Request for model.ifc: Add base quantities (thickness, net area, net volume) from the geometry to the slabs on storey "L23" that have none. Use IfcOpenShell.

First a look at what the model holds.

```python
import ifcopenshell
import ifcopenshell.util.element
import ifcopenshell.util.unit

model = ifcopenshell.open("model.ifc")
print(model.schema)
for unit_type in ("LENGTHUNIT", "AREAUNIT", "VOLUMEUNIT"):
    print(unit_type, ifcopenshell.util.unit.calculate_unit_scale(model, unit_type))
storey = next(s for s in model.by_type("IfcBuildingStorey") if s.Name == "L23")
slabs = [e for e in ifcopenshell.util.element.get_decomposition(storey) if e.is_a("IfcSlab")]
for e in sorted(slabs, key=lambda e: e.id()):
    print(e.id(), e.is_a(), e.Name, list(ifcopenshell.util.element.get_psets(e, qtos_only=True)), sep=" | ")
```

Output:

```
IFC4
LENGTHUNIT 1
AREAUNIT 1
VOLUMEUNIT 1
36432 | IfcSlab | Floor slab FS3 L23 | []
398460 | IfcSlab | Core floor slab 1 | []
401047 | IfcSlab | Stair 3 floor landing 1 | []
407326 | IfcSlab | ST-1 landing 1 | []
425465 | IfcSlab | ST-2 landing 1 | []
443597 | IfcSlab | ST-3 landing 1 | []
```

```python
import ifcopenshell
import ifcopenshell.api.pset
import ifcopenshell.geom
import ifcopenshell.util.element
import ifcopenshell.util.shape
import ifcopenshell.util.unit

model = ifcopenshell.open("model.ifc")
unit_scale = ifcopenshell.util.unit.calculate_unit_scale(model)
area_scale = ifcopenshell.util.unit.calculate_unit_scale(model, "AREAUNIT")
volume_scale = ifcopenshell.util.unit.calculate_unit_scale(model, "VOLUMEUNIT")
settings = ifcopenshell.geom.settings()

storey = next(s for s in model.by_type("IfcBuildingStorey") if s.Name == "L23")
slabs = [e for e in ifcopenshell.util.element.get_decomposition(storey) if e.is_a("IfcSlab")]

for e in sorted(slabs, key=lambda e: e.id()):
    if ifcopenshell.util.element.get_psets(e, qtos_only=True, should_inherit=False):
        continue
    # Geometry comes back in metres, in the element's own axes.
    shape = ifcopenshell.geom.create_shape(settings, e)
    values = {
        "Width": ifcopenshell.util.shape.get_z(shape.geometry) / unit_scale,
        "NetArea": ifcopenshell.util.shape.get_footprint_area(shape.geometry) / area_scale,
        "NetVolume": ifcopenshell.util.shape.get_volume(shape.geometry) / volume_scale,
    }
    qto = ifcopenshell.api.pset.add_qto(model, product=e, name="Qto_SlabBaseQuantities")
    ifcopenshell.api.pset.edit_qto(model, qto=qto, properties=values)
    print(e.id(), {k: round(v, 3) for k, v in values.items()})

model.write("model_rev.ifc")
```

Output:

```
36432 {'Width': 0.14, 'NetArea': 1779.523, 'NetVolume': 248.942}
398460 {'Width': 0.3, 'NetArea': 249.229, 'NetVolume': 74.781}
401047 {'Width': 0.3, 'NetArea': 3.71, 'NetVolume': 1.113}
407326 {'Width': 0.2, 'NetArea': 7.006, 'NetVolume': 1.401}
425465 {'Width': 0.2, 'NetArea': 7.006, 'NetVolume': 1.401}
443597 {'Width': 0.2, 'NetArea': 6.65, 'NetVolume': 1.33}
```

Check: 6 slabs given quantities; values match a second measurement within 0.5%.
